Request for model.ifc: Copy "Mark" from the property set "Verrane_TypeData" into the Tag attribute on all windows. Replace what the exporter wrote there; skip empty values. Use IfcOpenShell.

First a look at what the model holds.

```python
import ifcopenshell
import ifcopenshell.util.element

model = ifcopenshell.open("model.ifc")
print(model.schema)
windows = model.by_type("IfcWindow")
print(len(windows), "windows")
for e in windows[:8]:
    source = ifcopenshell.util.element.get_pset(e, "Verrane_TypeData", "Mark")
    target = e.Tag
    print(e.id(), repr(source), repr(target), sep=" | ")
```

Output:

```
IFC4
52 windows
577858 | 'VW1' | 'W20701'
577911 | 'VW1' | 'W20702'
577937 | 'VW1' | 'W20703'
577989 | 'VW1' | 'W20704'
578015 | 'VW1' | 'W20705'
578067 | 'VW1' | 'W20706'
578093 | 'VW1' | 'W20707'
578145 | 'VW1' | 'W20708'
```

```python
import ifcopenshell
import ifcopenshell.util.element

model = ifcopenshell.open("model.ifc")

count = 0
for e in model.by_type("IfcWindow"):
    value = ifcopenshell.util.element.get_pset(e, "Verrane_TypeData", "Mark")
    current = e.Tag
    if not value or not value.strip() or current == value:
        continue
    e.Tag = value
    count += 1

print(count, "windows updated")

model.write("model_updated.ifc")
```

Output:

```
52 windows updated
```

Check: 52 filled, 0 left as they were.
